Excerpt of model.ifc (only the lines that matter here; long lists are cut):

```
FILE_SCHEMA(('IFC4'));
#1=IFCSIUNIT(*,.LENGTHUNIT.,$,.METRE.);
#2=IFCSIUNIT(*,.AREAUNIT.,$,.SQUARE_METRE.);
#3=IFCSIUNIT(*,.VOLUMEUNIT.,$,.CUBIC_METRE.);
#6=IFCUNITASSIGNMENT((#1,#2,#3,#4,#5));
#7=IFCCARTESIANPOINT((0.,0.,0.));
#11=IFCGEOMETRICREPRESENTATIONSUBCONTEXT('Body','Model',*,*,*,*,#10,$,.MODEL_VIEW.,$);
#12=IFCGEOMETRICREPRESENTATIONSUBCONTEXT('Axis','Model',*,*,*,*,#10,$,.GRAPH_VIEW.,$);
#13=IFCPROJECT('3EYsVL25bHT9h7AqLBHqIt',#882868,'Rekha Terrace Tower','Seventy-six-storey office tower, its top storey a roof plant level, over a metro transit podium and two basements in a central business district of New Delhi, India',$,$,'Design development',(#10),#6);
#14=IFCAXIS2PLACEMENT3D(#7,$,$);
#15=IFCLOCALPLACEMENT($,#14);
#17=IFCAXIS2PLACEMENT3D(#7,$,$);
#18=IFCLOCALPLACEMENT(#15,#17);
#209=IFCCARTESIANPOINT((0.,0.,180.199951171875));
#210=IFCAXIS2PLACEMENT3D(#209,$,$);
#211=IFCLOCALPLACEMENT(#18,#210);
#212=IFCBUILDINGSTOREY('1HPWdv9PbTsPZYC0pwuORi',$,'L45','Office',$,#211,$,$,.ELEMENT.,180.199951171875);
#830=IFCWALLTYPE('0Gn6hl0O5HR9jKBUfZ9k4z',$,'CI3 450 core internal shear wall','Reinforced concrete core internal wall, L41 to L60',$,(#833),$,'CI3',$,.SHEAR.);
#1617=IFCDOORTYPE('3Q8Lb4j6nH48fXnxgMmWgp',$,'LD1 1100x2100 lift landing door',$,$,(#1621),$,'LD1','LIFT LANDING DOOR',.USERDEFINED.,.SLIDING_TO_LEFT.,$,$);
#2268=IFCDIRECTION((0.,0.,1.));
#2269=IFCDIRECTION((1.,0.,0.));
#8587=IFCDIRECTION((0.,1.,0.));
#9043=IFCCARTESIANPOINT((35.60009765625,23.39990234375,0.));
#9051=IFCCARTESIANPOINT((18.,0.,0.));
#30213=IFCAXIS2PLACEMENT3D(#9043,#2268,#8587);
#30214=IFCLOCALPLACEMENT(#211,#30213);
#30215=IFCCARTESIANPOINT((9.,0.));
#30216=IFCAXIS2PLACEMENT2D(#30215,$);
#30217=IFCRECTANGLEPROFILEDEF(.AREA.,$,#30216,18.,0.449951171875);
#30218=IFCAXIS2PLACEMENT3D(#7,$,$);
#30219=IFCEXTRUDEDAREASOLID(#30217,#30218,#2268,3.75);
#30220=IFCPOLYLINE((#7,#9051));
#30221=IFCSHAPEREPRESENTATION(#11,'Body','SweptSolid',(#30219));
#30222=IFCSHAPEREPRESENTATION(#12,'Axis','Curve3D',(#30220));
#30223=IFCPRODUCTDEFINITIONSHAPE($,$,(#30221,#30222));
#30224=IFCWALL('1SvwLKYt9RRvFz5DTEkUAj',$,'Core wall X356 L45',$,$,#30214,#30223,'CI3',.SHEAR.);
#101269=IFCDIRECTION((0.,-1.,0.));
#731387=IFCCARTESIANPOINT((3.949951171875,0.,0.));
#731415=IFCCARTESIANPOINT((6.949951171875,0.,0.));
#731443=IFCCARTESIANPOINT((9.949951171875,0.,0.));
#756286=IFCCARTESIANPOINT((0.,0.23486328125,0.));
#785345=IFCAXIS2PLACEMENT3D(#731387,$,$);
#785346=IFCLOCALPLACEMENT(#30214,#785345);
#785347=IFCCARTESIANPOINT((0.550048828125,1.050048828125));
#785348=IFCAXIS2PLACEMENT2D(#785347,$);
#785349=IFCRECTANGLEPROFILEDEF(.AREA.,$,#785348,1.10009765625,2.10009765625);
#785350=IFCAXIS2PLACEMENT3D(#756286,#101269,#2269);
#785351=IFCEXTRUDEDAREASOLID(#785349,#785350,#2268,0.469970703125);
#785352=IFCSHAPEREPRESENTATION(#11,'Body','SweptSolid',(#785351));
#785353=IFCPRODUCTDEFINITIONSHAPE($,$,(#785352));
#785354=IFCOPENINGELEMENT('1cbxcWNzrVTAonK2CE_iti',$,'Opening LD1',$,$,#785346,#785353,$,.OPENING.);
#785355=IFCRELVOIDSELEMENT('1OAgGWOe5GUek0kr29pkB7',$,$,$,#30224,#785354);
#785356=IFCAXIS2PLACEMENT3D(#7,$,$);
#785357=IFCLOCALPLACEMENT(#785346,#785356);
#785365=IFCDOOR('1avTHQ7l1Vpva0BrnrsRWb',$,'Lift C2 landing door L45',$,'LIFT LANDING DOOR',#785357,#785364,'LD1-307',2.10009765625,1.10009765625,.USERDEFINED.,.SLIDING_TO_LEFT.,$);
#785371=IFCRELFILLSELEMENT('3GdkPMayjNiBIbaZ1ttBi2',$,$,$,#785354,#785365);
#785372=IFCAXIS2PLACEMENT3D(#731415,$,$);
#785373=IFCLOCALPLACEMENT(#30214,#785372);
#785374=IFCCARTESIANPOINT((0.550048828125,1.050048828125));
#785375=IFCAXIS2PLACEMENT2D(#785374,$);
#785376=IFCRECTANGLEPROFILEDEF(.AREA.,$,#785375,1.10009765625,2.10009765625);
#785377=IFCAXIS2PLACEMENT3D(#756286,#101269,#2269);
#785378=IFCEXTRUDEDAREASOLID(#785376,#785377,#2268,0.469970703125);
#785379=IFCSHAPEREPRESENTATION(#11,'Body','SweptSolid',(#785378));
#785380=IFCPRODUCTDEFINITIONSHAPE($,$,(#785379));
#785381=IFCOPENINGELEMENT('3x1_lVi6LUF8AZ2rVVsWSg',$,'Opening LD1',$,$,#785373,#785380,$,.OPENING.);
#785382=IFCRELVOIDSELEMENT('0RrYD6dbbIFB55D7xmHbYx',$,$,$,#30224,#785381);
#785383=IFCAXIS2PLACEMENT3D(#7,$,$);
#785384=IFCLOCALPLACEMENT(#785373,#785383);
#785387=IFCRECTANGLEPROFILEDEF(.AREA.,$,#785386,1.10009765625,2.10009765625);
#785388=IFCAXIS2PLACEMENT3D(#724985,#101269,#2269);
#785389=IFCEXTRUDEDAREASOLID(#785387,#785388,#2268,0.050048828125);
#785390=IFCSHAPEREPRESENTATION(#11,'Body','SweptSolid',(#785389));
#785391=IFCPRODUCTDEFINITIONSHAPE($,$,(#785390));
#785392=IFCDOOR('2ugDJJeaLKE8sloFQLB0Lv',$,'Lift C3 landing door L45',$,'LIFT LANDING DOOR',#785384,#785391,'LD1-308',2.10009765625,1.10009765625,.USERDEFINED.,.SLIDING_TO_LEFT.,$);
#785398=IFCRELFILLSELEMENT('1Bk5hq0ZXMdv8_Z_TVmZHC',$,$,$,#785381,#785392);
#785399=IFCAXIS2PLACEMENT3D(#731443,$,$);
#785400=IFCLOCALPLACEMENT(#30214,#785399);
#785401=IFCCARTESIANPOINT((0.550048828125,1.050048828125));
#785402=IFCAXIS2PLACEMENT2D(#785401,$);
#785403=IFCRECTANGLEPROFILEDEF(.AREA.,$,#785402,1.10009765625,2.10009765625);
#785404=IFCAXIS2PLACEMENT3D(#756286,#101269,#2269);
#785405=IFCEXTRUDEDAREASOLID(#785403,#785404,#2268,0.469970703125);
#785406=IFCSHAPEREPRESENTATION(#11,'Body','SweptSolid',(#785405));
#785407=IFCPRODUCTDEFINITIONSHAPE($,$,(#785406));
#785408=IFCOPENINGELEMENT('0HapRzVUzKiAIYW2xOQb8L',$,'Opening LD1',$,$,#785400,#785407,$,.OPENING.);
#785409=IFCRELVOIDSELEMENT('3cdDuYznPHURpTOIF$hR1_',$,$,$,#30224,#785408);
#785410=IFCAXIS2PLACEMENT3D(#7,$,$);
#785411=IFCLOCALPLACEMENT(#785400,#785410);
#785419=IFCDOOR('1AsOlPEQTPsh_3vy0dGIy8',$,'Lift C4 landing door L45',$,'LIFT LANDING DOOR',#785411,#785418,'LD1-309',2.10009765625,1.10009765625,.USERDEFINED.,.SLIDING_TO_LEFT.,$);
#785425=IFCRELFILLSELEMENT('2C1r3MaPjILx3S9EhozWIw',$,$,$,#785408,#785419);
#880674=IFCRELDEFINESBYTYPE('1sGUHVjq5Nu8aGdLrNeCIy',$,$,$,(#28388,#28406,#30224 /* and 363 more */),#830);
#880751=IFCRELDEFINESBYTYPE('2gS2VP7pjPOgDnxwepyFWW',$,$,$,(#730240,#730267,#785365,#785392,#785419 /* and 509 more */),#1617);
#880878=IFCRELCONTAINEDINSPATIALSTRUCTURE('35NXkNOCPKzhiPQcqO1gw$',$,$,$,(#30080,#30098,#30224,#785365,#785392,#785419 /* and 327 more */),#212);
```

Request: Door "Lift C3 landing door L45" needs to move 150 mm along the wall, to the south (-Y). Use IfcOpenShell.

```python
import ifcopenshell
import ifcopenshell.api.geometry
import ifcopenshell.util.placement

model = ifcopenshell.open("model.ifc")

door = model.by_guid("2ugDJJeaLKE8sloFQLB0Lv")
opening = door.FillsVoids[0].RelatingOpeningElement
wall = opening.VoidsElements[0].RelatingBuildingElement

wall_matrix = ifcopenshell.util.placement.get_local_placement(wall.ObjectPlacement)
shift = wall_matrix[:3, 0] * -0.15
before = ifcopenshell.util.placement.get_local_placement(door.ObjectPlacement)[:3, 3].copy()

# The door is placed relative to its opening, so it follows when the opening moves.
matrix = ifcopenshell.util.placement.get_local_placement(opening.ObjectPlacement)
matrix[:3, 3] += shift
ifcopenshell.api.geometry.edit_object_placement(
    model, product=opening, matrix=matrix, is_si=False, should_transform_children=True
)

after = ifcopenshell.util.placement.get_local_placement(door.ObjectPlacement)[:3, 3]
print("door moved by", (after - before).round(3) + 0.0)

model.write("model_rev.ifc")
```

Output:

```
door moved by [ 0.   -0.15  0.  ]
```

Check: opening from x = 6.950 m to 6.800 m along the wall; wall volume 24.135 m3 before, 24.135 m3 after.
